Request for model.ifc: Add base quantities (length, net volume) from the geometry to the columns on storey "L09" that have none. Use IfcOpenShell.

First a look at what the model holds.

```python
import ifcopenshell
import ifcopenshell.util.element
import ifcopenshell.util.unit

model = ifcopenshell.open("model.ifc")
print(model.schema)
for unit_type in ("LENGTHUNIT", "AREAUNIT", "VOLUMEUNIT"):
    print(unit_type, ifcopenshell.util.unit.calculate_unit_scale(model, unit_type))
storey = next(s for s in model.by_type("IfcBuildingStorey") if s.Name == "L09")
columns = [e for e in ifcopenshell.util.element.get_decomposition(storey) if e.is_a("IfcColumn")]
for e in sorted(columns, key=lambda e: e.id()):
    print(e.id(), e.is_a(), e.Name, list(ifcopenshell.util.element.get_psets(e, qtos_only=True)), sep=" | ")
```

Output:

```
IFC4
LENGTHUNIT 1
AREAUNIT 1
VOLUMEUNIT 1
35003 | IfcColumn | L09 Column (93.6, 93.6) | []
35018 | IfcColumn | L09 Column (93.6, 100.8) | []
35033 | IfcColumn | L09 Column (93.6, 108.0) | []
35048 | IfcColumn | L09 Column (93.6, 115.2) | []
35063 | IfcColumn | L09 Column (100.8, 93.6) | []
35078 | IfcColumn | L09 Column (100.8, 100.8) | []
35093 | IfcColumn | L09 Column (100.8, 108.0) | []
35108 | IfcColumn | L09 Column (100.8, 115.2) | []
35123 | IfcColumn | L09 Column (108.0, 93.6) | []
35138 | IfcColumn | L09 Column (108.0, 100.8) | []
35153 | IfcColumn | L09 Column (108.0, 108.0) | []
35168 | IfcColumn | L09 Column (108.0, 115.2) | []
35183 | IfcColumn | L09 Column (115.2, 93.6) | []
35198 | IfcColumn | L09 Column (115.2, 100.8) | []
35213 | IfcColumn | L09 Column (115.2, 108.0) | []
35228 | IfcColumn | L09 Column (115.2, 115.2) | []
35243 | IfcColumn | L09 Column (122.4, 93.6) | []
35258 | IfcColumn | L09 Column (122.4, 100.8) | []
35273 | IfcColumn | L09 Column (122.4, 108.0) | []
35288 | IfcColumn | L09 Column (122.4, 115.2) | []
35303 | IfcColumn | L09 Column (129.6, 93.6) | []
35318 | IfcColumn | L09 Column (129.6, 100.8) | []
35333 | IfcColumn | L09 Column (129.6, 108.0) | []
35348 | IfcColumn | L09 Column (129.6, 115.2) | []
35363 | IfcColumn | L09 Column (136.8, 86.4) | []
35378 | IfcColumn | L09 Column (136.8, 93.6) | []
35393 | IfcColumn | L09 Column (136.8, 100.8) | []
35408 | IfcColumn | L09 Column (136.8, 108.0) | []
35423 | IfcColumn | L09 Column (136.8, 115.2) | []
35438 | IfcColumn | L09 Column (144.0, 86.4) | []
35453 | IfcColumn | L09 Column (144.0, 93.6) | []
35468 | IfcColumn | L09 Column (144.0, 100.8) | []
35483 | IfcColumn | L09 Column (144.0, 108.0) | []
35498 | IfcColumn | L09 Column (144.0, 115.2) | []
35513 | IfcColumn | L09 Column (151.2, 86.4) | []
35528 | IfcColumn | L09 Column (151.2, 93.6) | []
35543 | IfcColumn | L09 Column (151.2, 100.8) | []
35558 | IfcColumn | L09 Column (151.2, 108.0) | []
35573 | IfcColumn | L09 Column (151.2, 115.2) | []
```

```python
import ifcopenshell
import ifcopenshell.api.pset
import ifcopenshell.geom
import ifcopenshell.util.element
import ifcopenshell.util.shape
import ifcopenshell.util.unit

model = ifcopenshell.open("model.ifc")
unit_scale = ifcopenshell.util.unit.calculate_unit_scale(model)
volume_scale = ifcopenshell.util.unit.calculate_unit_scale(model, "VOLUMEUNIT")
settings = ifcopenshell.geom.settings()

storey = next(s for s in model.by_type("IfcBuildingStorey") if s.Name == "L09")
columns = [e for e in ifcopenshell.util.element.get_decomposition(storey) if e.is_a("IfcColumn")]

for e in sorted(columns, key=lambda e: e.id()):
    if ifcopenshell.util.element.get_psets(e, qtos_only=True, should_inherit=False):
        continue
    # Geometry comes back in metres, in the element's own axes.
    shape = ifcopenshell.geom.create_shape(settings, e)
    values = {
        "Length": ifcopenshell.util.shape.get_z(shape.geometry) / unit_scale,
        "NetVolume": ifcopenshell.util.shape.get_volume(shape.geometry) / volume_scale,
    }
    qto = ifcopenshell.api.pset.add_qto(model, product=e, name="Qto_ColumnBaseQuantities")
    ifcopenshell.api.pset.edit_qto(model, qto=qto, properties=values)
    print(e.id(), {k: round(v, 3) for k, v in values.items()})

model.write("model_edited.ifc")
```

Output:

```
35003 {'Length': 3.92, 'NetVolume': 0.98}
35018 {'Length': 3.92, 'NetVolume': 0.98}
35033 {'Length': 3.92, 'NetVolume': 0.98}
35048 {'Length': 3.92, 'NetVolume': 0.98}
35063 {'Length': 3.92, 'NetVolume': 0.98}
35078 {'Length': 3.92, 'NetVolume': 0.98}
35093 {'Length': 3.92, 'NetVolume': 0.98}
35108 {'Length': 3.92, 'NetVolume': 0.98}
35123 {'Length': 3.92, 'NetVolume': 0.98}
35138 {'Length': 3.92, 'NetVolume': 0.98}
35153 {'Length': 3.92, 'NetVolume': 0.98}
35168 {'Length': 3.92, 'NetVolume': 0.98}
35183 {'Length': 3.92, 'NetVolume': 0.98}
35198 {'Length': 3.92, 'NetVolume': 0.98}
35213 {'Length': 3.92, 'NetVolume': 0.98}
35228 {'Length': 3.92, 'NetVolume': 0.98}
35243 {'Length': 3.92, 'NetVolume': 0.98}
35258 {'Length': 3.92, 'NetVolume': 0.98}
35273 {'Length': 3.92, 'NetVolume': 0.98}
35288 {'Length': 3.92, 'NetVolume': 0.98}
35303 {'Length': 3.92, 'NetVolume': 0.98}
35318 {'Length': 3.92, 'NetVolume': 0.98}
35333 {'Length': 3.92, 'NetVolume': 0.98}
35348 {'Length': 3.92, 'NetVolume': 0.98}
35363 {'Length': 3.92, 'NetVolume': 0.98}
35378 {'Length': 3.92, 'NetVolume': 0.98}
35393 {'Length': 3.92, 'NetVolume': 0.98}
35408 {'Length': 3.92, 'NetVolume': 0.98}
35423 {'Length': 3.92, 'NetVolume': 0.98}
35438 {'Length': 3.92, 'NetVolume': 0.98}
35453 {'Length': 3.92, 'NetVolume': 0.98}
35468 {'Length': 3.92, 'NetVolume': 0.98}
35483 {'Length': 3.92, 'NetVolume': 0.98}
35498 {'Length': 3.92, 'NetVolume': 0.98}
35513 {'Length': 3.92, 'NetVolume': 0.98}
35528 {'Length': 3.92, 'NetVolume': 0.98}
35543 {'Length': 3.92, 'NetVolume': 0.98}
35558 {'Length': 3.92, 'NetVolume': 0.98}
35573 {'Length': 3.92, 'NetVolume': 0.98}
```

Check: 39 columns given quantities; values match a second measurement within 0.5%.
